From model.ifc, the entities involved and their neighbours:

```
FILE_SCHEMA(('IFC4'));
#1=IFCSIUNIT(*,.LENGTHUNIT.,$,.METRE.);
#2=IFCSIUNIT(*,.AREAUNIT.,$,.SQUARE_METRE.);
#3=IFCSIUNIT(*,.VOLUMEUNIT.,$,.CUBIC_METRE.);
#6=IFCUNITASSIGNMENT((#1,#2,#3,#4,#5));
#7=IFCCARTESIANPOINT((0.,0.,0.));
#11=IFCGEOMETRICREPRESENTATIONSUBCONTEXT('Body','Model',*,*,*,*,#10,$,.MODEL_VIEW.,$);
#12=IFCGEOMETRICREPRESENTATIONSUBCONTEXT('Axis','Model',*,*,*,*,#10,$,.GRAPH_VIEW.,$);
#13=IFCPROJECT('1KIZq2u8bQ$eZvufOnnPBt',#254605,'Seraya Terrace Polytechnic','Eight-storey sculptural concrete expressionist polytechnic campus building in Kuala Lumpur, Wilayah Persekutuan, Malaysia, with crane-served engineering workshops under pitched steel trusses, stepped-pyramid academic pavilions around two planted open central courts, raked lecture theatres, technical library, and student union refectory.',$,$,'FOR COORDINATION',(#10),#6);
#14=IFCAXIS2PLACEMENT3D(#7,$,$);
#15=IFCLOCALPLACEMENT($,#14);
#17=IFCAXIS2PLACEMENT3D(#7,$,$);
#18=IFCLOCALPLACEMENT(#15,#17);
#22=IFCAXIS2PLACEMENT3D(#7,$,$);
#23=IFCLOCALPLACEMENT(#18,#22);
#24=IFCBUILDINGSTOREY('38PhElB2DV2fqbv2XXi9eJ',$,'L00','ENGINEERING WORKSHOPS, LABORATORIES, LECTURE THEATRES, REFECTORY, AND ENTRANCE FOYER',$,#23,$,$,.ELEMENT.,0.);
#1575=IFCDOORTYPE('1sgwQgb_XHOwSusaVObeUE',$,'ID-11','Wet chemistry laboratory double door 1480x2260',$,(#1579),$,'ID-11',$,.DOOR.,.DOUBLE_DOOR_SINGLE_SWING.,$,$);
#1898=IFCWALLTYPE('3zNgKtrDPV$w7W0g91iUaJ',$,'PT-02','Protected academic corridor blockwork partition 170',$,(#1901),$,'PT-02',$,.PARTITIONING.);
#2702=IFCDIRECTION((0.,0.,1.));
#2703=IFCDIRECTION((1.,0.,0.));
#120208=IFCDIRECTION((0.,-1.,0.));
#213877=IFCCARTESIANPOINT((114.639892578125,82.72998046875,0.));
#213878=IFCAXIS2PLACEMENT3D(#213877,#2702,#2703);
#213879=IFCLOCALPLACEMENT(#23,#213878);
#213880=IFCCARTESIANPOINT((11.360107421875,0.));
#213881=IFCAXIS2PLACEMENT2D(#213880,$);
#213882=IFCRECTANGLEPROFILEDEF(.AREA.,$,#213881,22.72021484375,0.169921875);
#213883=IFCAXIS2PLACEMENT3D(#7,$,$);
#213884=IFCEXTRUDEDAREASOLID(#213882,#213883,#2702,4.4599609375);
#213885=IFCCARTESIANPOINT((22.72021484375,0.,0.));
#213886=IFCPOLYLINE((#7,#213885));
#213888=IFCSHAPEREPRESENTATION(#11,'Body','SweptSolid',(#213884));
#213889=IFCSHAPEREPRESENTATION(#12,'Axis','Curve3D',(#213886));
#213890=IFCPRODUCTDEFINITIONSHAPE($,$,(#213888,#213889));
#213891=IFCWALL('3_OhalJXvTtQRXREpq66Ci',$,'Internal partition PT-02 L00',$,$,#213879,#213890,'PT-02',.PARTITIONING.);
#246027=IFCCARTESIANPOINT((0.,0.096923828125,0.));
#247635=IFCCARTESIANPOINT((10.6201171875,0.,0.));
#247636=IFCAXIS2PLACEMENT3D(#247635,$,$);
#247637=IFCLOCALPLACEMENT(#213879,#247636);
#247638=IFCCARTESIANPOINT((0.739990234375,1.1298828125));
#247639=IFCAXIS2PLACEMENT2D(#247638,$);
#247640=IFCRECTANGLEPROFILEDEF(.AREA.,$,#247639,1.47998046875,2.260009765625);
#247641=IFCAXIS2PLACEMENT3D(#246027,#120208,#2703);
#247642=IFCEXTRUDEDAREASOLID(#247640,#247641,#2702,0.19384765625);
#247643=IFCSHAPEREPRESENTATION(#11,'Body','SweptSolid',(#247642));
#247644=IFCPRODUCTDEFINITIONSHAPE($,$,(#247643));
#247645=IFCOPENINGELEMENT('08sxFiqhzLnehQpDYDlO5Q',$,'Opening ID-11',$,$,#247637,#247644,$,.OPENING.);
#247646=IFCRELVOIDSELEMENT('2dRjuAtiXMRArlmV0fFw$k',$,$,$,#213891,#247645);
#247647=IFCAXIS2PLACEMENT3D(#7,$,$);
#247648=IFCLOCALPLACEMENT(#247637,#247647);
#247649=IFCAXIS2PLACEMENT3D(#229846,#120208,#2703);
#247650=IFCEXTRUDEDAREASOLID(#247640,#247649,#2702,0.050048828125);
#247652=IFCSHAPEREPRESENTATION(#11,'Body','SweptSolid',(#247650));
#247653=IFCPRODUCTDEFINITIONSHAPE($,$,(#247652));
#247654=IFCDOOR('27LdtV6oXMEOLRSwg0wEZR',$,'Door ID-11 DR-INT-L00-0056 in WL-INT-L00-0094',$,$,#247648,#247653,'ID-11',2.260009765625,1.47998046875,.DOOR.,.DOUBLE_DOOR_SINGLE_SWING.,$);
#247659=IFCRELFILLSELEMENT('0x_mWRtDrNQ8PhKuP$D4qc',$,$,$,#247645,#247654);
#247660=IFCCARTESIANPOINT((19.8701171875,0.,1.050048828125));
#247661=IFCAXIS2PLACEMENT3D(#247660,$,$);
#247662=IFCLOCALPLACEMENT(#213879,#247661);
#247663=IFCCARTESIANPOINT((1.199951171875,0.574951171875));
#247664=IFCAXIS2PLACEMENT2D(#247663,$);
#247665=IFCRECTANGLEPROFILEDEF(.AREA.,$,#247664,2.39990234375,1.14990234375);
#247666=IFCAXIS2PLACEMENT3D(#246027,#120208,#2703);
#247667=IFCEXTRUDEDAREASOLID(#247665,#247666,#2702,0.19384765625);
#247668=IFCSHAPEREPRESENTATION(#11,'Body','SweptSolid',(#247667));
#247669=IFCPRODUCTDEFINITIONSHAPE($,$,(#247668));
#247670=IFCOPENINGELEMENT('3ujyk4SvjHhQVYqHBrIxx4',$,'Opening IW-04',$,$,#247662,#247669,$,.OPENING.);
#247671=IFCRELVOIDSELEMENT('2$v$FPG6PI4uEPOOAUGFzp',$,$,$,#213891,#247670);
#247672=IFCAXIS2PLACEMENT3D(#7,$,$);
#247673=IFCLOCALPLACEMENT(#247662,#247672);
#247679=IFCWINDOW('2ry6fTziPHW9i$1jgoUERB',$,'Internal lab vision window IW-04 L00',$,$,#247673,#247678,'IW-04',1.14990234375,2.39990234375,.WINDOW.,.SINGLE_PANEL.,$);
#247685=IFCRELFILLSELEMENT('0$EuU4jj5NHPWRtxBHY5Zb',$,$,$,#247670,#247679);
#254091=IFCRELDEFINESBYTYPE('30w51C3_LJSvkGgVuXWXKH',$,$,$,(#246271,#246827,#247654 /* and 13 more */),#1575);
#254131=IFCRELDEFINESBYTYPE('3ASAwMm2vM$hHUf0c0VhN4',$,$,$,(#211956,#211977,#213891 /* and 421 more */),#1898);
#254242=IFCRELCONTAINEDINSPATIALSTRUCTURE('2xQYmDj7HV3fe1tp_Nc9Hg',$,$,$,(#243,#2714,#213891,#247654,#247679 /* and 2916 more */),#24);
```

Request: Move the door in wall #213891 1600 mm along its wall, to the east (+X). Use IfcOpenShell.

```python
import ifcopenshell
import ifcopenshell.api.geometry
import ifcopenshell.util.placement

model = ifcopenshell.open("model.ifc")

door = model.by_guid("27LdtV6oXMEOLRSwg0wEZR")
opening = door.FillsVoids[0].RelatingOpeningElement
wall = opening.VoidsElements[0].RelatingBuildingElement

wall_matrix = ifcopenshell.util.placement.get_local_placement(wall.ObjectPlacement)
shift = wall_matrix[:3, 0] * 1.6
before = ifcopenshell.util.placement.get_local_placement(door.ObjectPlacement)[:3, 3].copy()

# The door is placed relative to its opening, so it follows when the opening moves.
matrix = ifcopenshell.util.placement.get_local_placement(opening.ObjectPlacement)
matrix[:3, 3] += shift
ifcopenshell.api.geometry.edit_object_placement(
    model, product=opening, matrix=matrix, is_si=False, should_transform_children=True
)

after = ifcopenshell.util.placement.get_local_placement(door.ObjectPlacement)[:3, 3]
print("door moved by", (after - before).round(3) + 0.0)

model.write("model_updated.ifc")
```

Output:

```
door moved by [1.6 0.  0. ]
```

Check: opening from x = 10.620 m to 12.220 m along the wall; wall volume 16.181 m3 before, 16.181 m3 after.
